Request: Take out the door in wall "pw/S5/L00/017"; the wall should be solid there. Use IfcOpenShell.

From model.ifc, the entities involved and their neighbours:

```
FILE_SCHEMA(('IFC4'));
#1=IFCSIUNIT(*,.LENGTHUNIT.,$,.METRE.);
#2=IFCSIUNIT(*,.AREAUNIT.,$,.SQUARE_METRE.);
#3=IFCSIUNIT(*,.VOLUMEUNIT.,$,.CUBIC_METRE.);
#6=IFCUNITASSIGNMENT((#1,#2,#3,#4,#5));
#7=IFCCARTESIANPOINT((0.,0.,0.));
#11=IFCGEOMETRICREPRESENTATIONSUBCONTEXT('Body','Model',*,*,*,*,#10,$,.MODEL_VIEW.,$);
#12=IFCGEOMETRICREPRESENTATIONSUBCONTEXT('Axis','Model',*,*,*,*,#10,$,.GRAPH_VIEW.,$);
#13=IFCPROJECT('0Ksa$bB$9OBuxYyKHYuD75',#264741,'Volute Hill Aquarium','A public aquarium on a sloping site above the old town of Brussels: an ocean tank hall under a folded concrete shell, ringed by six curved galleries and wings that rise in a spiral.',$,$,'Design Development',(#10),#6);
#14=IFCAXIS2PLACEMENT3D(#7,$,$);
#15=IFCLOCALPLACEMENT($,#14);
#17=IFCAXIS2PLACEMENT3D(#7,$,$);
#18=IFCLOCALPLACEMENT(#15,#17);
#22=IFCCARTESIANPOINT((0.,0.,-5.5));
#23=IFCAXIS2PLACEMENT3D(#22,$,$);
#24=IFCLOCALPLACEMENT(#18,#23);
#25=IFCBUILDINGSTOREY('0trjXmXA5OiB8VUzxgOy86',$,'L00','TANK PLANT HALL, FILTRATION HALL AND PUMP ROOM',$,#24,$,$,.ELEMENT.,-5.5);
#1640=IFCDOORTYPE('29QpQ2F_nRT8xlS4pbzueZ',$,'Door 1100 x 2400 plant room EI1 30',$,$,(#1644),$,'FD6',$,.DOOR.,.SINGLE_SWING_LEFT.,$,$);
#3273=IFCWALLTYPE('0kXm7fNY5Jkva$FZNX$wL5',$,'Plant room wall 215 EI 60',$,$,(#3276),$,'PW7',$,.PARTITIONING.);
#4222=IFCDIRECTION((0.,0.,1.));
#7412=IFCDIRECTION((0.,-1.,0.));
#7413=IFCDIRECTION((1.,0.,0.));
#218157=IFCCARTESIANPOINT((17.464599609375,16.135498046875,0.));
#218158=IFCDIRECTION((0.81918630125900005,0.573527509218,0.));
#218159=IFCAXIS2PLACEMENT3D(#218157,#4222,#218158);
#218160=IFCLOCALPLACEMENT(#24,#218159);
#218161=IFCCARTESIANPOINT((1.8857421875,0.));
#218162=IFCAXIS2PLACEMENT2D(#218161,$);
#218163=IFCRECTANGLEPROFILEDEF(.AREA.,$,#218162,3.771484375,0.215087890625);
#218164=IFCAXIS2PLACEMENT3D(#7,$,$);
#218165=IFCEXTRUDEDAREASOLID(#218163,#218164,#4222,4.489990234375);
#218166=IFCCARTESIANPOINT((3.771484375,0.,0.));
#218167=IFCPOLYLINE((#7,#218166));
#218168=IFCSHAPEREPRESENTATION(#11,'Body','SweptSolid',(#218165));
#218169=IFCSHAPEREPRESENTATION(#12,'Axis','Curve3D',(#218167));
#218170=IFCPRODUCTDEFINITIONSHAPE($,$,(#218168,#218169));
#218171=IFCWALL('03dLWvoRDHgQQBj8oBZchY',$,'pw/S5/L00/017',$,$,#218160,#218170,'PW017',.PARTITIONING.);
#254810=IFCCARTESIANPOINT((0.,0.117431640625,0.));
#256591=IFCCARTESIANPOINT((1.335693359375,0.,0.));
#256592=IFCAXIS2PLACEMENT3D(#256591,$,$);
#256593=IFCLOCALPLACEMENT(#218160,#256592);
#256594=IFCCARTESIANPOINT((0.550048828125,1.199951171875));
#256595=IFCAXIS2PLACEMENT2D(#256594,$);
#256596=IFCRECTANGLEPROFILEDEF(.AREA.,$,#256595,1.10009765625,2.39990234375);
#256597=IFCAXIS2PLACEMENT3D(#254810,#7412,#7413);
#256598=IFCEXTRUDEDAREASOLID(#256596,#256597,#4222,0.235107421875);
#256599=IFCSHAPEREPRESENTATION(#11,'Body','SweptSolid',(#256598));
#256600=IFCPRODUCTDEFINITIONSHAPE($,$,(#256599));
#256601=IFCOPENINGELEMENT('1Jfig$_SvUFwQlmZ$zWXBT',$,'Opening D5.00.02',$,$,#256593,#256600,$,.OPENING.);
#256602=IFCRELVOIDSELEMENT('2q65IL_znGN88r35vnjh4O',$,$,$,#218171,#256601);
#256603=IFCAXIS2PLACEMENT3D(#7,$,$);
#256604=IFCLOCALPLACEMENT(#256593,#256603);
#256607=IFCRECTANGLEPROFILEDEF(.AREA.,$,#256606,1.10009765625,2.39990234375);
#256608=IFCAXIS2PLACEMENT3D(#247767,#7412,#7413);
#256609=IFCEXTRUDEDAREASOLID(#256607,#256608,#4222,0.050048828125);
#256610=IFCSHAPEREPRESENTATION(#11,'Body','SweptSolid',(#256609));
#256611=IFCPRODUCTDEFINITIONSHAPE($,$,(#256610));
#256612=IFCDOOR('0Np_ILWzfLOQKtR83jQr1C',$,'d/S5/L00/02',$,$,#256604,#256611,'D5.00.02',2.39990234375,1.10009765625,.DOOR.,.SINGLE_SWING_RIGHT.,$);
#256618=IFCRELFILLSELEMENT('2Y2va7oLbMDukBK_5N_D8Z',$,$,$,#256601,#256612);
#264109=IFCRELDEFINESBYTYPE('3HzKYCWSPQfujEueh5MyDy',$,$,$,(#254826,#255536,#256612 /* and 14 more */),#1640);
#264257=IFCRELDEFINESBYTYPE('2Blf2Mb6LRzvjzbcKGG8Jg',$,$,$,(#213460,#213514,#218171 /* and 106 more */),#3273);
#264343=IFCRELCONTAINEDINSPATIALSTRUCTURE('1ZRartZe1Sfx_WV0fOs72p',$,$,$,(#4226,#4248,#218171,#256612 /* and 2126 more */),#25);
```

```python
import ifcopenshell
import ifcopenshell.api.feature
import ifcopenshell.api.root
import ifcopenshell.geom
import ifcopenshell.util.shape

model = ifcopenshell.open("model.ifc")
settings = ifcopenshell.geom.settings()


def volume(element):
    """Net volume in cubic metres, openings subtracted."""
    shape = ifcopenshell.geom.create_shape(settings, element)
    return ifcopenshell.util.shape.get_volume(shape.geometry)


door = model.by_id(256612)
opening = door.FillsVoids[0].RelatingOpeningElement
wall = opening.VoidsElements[0].RelatingBuildingElement
before = volume(wall)

ifcopenshell.api.root.remove_product(model, product=door)
ifcopenshell.api.feature.remove_feature(model, feature=opening)

after = volume(wall)

print(f"wall volume {before:.3f} -> {after:.3f} m3")

model.write("model_v2.ifc")
```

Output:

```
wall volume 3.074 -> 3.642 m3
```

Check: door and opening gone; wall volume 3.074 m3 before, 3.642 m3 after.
